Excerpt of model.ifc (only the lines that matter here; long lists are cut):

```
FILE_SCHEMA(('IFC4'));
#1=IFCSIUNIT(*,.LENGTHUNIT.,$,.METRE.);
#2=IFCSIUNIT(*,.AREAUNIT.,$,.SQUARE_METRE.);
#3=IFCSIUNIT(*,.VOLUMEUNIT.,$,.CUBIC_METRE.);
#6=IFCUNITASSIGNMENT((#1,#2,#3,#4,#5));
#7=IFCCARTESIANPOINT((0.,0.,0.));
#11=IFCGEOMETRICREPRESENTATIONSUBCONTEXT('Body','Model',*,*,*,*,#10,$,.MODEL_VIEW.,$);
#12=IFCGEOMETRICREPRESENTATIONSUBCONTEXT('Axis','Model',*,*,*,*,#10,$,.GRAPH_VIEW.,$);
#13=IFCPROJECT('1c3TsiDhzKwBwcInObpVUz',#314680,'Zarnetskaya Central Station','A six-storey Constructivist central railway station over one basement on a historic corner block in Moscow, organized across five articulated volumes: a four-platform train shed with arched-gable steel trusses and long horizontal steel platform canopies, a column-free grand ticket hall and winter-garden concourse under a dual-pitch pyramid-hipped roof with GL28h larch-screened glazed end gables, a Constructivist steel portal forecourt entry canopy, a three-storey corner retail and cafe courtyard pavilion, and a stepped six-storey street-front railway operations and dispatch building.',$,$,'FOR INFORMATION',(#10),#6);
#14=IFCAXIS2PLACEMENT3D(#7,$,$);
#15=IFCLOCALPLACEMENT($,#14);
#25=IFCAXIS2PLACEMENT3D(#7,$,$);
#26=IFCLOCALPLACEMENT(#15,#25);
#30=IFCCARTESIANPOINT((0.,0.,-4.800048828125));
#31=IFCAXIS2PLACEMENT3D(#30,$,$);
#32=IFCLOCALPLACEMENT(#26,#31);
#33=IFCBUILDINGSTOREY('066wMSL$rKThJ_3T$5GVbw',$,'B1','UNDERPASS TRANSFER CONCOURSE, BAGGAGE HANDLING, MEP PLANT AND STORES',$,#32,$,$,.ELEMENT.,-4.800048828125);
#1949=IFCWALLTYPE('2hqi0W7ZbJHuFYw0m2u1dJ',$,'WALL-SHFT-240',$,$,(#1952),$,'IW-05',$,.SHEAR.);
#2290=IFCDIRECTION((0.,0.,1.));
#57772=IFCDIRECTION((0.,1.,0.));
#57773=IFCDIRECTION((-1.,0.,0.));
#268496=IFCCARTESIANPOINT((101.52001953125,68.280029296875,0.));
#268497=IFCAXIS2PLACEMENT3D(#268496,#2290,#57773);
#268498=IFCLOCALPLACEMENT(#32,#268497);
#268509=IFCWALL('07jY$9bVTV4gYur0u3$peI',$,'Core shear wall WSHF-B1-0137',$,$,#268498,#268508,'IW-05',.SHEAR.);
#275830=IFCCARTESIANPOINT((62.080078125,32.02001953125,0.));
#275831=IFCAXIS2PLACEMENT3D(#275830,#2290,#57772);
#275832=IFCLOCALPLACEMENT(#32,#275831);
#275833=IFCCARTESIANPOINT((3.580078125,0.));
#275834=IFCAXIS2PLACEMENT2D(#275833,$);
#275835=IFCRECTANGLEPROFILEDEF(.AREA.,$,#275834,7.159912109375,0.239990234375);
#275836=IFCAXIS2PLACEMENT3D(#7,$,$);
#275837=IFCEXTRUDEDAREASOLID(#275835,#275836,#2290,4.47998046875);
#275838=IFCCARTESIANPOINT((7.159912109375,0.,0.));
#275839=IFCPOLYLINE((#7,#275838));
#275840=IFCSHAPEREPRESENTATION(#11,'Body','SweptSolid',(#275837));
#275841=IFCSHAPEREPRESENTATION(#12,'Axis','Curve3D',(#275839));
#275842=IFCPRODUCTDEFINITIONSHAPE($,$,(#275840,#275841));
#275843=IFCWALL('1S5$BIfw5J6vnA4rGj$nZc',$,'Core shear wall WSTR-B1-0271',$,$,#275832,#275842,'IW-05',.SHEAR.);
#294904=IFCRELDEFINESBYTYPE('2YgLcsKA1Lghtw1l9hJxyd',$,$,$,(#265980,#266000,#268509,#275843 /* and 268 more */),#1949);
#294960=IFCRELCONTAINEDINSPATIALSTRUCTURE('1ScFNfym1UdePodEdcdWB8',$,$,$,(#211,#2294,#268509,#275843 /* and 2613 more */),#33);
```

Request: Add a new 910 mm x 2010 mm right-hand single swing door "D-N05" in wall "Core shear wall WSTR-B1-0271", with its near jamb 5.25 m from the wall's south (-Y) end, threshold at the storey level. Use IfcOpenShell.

```python
import numpy as np
import ifcopenshell
import ifcopenshell.api.feature
import ifcopenshell.api.geometry
import ifcopenshell.api.root
import ifcopenshell.api.spatial
import ifcopenshell.geom
import ifcopenshell.util.element
import ifcopenshell.util.placement
import ifcopenshell.util.representation
import ifcopenshell.util.shape
import ifcopenshell.util.unit

model = ifcopenshell.open("model.ifc")
unit_scale = ifcopenshell.util.unit.calculate_unit_scale(model)
settings = ifcopenshell.geom.settings()


def volume(element):
    """Net volume in cubic metres, openings subtracted."""
    shape = ifcopenshell.geom.create_shape(settings, element)
    return ifcopenshell.util.shape.get_volume(shape.geometry)


wall = model.by_guid("1S5$BIfw5J6vnA4rGj$nZc")
storey = ifcopenshell.util.element.get_container(wall, ifc_class="IfcBuildingStorey")
context = ifcopenshell.util.representation.get_context(model, "Model", "Body", "MODEL_VIEW")
before = volume(wall)

width, height, from_end, sill = 0.91, 2.01, 5.25, 0.0  # metres

# The wall runs along its own X axis, and the end named is its -X end.
wall_shape = ifcopenshell.geom.create_shape(settings, wall)
x, y, z = ifcopenshell.util.shape.get_vertices(wall_shape.geometry).T
start = x.min() + from_end
face, thickness = float(y.min()), float(y.max() - y.min())
wall_matrix = ifcopenshell.util.placement.get_local_placement(wall.ObjectPlacement)
level = ifcopenshell.util.placement.get_local_placement(storey.ObjectPlacement)[2, 3]


def in_wall(x, y):
    """Placement at x, y metres in the wall's axes, at sill height."""
    matrix = wall_matrix.copy()
    matrix[:, 3] = wall_matrix @ np.array([x / unit_scale, y / unit_scale, 0.0, 1.0])
    matrix[2, 3] = level + sill / unit_scale
    return matrix


# Opening: a box that overshoots both wall faces by 50 mm.
opening = ifcopenshell.api.root.create_entity(model, ifc_class="IfcOpeningElement", predefined_type="OPENING")
box = ifcopenshell.api.geometry.add_wall_representation(
    model, context=context, length=width, height=height, thickness=thickness + 0.1
)
ifcopenshell.api.geometry.assign_representation(model, product=opening, representation=box)
ifcopenshell.api.geometry.edit_object_placement(model, product=opening, matrix=in_wall(start, face - 0.05), is_si=False)
ifcopenshell.api.feature.add_feature(model, feature=opening, element=wall)

door = ifcopenshell.api.root.create_entity(model, ifc_class="IfcDoor", name="D-N05", predefined_type="DOOR")
door.OverallWidth, door.OverallHeight = width / unit_scale, height / unit_scale
door.OperationType = "SINGLE_SWING_RIGHT"
body = ifcopenshell.api.geometry.add_door_representation(
    model,
    context=context,
    overall_width=door.OverallWidth,
    overall_height=door.OverallHeight,
    operation_type="SINGLE_SWING_RIGHT",
    lining_properties={"LiningDepth": thickness / unit_scale, "ThresholdDepth": thickness / unit_scale},
)
ifcopenshell.api.geometry.assign_representation(model, product=door, representation=body)
ifcopenshell.api.spatial.assign_container(model, products=[door], relating_structure=storey)
ifcopenshell.api.feature.add_filling(model, opening=opening, element=door)

# The lining spans the wall, so the door starts at the wall face.
ifcopenshell.api.geometry.edit_object_placement(model, product=door, matrix=in_wall(start, face), is_si=False)

after = volume(wall)

print(f"wall volume {before:.3f} -> {after:.3f} m3")

model.write("model_edited.ifc")
```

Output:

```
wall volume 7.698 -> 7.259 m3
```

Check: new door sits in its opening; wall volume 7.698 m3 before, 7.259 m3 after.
